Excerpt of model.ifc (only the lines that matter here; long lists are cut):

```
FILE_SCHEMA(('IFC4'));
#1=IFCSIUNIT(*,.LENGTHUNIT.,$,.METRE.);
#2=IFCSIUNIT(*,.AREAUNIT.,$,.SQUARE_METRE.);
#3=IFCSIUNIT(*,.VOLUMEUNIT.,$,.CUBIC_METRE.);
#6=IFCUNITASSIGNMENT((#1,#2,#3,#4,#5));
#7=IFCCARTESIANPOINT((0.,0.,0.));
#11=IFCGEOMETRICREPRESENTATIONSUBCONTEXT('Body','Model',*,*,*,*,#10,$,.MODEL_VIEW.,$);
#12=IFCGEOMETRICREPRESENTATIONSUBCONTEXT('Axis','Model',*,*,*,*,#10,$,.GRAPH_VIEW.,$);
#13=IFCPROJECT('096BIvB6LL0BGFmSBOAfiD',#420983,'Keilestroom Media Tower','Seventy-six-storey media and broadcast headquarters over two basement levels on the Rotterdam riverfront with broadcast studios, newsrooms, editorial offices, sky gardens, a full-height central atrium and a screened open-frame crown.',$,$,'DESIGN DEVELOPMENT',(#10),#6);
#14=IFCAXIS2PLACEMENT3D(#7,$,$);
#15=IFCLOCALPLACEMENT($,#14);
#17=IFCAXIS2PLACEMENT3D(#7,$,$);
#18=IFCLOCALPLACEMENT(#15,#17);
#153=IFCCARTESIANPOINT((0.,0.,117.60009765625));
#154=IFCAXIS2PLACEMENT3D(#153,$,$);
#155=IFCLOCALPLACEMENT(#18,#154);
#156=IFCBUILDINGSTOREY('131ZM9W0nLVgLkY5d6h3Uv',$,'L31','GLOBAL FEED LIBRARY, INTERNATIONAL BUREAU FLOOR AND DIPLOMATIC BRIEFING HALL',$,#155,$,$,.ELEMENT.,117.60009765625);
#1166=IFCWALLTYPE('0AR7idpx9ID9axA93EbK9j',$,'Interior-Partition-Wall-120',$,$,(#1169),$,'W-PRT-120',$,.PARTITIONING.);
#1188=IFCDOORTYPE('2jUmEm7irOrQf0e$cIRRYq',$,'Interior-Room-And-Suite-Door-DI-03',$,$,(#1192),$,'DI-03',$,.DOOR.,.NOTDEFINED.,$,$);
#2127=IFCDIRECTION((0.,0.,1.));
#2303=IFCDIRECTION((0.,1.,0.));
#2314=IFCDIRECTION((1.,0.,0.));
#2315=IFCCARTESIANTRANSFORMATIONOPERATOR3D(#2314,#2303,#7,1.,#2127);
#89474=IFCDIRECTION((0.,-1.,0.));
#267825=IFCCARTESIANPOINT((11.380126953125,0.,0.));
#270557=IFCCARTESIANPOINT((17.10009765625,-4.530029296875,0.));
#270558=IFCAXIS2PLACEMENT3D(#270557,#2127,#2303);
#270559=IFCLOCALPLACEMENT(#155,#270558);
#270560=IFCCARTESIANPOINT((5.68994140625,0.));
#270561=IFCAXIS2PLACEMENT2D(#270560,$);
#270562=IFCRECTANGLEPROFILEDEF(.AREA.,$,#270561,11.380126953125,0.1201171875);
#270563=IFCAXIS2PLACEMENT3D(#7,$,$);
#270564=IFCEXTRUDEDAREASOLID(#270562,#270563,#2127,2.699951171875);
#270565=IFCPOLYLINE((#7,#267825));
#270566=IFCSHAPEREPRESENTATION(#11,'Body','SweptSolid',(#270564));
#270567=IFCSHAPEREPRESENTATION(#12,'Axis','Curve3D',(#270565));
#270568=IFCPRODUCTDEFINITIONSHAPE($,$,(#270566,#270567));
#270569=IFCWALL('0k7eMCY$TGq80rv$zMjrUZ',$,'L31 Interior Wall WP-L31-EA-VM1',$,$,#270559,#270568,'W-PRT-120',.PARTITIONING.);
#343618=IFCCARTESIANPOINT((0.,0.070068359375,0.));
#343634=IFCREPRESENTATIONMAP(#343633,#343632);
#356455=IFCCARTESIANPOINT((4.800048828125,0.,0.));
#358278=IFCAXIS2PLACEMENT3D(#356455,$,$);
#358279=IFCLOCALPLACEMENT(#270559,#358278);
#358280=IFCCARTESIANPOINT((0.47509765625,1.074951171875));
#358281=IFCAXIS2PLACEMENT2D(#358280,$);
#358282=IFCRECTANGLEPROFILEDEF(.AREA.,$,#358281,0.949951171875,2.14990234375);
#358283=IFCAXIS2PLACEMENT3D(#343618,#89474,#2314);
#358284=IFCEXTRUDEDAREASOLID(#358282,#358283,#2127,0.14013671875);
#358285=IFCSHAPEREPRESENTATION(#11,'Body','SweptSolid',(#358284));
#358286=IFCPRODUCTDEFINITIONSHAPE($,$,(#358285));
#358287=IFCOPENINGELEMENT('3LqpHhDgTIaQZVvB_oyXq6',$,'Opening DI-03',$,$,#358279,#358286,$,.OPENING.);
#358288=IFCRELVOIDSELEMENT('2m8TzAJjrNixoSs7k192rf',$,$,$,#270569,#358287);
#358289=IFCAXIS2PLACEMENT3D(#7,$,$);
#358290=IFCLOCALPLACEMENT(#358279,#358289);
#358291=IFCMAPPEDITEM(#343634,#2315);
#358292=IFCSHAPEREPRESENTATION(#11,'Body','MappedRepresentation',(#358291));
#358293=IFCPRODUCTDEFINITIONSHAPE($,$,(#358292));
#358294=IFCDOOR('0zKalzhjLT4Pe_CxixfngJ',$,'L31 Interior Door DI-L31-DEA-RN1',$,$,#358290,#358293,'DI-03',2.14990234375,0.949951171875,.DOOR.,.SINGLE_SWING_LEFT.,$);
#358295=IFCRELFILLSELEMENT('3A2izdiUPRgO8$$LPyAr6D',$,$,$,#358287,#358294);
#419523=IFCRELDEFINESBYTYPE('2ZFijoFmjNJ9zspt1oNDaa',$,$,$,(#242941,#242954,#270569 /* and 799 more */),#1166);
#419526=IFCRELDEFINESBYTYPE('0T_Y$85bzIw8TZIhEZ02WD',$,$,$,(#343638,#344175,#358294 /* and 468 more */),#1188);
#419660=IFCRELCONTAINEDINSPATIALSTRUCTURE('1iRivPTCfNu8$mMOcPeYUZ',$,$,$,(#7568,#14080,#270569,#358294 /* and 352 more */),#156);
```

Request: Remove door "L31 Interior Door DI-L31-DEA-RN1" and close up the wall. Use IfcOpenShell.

```python
import ifcopenshell
import ifcopenshell.api.feature
import ifcopenshell.api.root
import ifcopenshell.geom
import ifcopenshell.util.shape

model = ifcopenshell.open("model.ifc")
settings = ifcopenshell.geom.settings()


def volume(element):
    """Net volume in cubic metres, openings subtracted."""
    shape = ifcopenshell.geom.create_shape(settings, element)
    return ifcopenshell.util.shape.get_volume(shape.geometry)


door = model.by_id(358294)
opening = door.FillsVoids[0].RelatingOpeningElement
wall = opening.VoidsElements[0].RelatingBuildingElement
before = volume(wall)

ifcopenshell.api.root.remove_product(model, product=door)
ifcopenshell.api.feature.remove_feature(model, feature=opening)

after = volume(wall)

print(f"wall volume {before:.3f} -> {after:.3f} m3")

model.write("model_edited.ifc")
```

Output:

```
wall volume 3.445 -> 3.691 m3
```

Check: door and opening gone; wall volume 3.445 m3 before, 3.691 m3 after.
